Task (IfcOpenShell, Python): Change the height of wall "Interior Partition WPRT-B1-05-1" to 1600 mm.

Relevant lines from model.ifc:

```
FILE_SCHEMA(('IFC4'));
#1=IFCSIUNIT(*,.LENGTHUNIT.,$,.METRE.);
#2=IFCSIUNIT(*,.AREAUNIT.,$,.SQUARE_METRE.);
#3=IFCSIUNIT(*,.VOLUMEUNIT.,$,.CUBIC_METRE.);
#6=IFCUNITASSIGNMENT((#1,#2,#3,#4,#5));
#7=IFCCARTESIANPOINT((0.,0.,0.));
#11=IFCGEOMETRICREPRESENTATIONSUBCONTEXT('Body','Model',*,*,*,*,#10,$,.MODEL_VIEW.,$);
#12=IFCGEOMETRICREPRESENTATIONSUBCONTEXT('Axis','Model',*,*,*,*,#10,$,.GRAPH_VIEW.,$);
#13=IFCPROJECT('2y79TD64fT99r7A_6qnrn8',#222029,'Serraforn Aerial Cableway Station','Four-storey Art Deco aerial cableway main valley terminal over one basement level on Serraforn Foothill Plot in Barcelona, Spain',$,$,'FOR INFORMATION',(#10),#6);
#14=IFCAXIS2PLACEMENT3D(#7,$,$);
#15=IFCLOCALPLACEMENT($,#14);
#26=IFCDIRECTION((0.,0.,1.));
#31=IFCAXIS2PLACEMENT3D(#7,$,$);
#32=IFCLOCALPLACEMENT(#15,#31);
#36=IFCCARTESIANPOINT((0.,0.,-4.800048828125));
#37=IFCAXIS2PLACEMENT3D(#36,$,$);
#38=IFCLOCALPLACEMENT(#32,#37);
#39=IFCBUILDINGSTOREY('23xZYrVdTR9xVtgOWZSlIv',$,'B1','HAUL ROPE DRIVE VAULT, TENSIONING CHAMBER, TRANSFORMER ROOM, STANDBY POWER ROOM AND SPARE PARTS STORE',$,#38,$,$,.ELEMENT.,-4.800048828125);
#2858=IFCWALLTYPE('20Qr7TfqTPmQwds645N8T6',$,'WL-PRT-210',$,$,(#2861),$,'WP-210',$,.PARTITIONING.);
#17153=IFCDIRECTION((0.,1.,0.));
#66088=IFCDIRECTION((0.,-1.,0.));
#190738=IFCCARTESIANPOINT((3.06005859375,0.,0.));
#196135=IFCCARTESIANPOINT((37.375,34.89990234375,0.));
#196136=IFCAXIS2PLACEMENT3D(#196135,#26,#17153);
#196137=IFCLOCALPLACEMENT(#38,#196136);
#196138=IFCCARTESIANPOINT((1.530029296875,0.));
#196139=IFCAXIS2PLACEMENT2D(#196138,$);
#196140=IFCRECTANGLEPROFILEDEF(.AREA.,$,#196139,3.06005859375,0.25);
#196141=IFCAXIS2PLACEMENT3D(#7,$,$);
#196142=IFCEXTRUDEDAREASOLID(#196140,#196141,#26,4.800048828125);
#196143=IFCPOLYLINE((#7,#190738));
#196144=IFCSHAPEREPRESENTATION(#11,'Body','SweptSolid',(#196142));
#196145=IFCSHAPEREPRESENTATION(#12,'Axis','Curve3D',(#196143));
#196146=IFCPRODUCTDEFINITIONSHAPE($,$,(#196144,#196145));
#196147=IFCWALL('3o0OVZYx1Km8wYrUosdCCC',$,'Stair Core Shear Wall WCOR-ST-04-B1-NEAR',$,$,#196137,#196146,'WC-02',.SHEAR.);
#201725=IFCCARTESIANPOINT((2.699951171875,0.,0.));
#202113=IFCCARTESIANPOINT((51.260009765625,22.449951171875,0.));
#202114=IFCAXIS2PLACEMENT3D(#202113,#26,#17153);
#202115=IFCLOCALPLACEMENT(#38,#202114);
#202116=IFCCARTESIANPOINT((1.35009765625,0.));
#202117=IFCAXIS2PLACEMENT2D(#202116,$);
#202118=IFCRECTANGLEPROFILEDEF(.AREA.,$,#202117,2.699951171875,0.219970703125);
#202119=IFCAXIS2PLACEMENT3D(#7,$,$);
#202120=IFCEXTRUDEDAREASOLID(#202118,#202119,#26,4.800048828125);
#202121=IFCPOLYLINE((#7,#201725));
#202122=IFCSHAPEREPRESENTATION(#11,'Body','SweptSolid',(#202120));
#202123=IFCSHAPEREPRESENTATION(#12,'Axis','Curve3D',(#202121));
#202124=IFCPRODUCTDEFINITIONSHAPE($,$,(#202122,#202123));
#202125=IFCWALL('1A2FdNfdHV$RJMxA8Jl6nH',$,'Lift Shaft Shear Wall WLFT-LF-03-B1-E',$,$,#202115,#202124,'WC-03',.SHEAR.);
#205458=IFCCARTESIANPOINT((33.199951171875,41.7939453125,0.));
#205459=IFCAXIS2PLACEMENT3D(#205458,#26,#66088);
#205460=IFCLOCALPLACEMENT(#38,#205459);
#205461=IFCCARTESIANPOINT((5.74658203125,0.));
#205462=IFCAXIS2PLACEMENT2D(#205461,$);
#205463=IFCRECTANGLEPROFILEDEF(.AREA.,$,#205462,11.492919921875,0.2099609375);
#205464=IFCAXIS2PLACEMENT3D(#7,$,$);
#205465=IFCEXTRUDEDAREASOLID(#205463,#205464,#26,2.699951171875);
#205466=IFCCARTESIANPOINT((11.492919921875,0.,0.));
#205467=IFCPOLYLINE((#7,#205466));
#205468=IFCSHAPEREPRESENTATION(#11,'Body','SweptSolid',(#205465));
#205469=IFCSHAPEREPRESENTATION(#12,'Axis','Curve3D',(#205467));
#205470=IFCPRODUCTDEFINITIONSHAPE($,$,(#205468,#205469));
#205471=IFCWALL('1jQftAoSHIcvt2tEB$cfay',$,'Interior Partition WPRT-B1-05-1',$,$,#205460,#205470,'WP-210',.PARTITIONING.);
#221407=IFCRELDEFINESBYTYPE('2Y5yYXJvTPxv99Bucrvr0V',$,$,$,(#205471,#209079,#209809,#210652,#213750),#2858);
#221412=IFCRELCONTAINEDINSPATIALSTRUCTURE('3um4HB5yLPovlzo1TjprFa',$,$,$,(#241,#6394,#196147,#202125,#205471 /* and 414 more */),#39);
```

```python
import ifcopenshell
import ifcopenshell.geom
import ifcopenshell.util.representation
import ifcopenshell.util.shape
import ifcopenshell.util.unit

model = ifcopenshell.open("model.ifc")
unit_scale = ifcopenshell.util.unit.calculate_unit_scale(model)
settings = ifcopenshell.geom.settings()


def volume(element):
    """Net volume in cubic metres, openings subtracted."""
    shape = ifcopenshell.geom.create_shape(settings, element)
    return ifcopenshell.util.shape.get_volume(shape.geometry)


wall = model.by_guid("1jQftAoSHIcvt2tEB$cfay")
before = volume(wall)

body = ifcopenshell.util.representation.get_representation(wall, "Model", "Body")
solid = body.Items[0]
old_height = solid.Depth
solid.Depth = 1.6 / unit_scale
after = volume(wall)

print(f"height {old_height:g} -> {solid.Depth:g}, volume {before:.3f} -> {after:.3f} m3")

model.write("model_v2.ifc")
```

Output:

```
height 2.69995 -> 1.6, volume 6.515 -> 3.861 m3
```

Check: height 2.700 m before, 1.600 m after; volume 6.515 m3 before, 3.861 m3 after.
